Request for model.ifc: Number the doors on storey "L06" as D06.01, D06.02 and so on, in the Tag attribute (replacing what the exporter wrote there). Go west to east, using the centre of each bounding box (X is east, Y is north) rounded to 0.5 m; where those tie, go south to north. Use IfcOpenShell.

First a look at what the model holds.

```python
import ifcopenshell
import ifcopenshell.util.element
import ifcopenshell.util.placement

model = ifcopenshell.open("model.ifc")
print(model.schema)
storey = next(s for s in model.by_type("IfcBuildingStorey") if s.Name == "L06")
doors = [e for e in ifcopenshell.util.element.get_decomposition(storey) if e.is_a("IfcDoor")]
for e in sorted(doors, key=lambda e: e.id()):
    origin = ifcopenshell.util.placement.get_local_placement(e.ObjectPlacement)[:3, 3]
    print(e.id(), e.Tag, e.Name, origin.round(2) + 0.0, sep=" | ")
```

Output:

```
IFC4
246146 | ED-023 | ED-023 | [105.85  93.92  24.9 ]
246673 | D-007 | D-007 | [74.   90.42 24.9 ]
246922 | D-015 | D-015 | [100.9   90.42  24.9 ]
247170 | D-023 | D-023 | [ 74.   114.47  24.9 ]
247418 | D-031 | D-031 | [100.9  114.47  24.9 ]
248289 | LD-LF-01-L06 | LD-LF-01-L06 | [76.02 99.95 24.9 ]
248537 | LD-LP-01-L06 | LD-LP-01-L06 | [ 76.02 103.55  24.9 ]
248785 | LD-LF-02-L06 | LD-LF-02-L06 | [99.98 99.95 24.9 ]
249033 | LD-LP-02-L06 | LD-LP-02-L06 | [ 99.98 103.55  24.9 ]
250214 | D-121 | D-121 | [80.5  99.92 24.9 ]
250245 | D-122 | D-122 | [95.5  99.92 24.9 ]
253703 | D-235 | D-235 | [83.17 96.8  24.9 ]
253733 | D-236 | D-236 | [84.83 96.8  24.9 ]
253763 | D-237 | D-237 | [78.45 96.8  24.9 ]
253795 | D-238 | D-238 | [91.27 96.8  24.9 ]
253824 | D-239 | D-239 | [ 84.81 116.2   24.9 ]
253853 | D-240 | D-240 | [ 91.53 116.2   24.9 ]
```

```python
import ifcopenshell
import ifcopenshell.geom
import ifcopenshell.util.element
import ifcopenshell.util.shape

model = ifcopenshell.open("model.ifc")
settings = ifcopenshell.geom.settings()
settings.set("use-world-coords", True)


def centre(element):
    shape = ifcopenshell.geom.create_shape(settings, element)
    return ifcopenshell.util.shape.get_bbox_centroid(shape.geometry)


storey = next(s for s in model.by_type("IfcBuildingStorey") if s.Name == "L06")
doors = [e for e in ifcopenshell.util.element.get_decomposition(storey) if e.is_a("IfcDoor")]

# Insertion points can sit at a corner or the storey origin, so sort by the geometry (in metres).
centres = {e: centre(e) for e in doors}
doors.sort(key=lambda e: (round(centres[e][0] / 0.5), centres[e][1]))

for i, e in enumerate(doors, start=1):
    number = f"D06.{i:02d}"
    e.Tag = number
    print(e.id(), number)

model.write("model-out.ifc")
```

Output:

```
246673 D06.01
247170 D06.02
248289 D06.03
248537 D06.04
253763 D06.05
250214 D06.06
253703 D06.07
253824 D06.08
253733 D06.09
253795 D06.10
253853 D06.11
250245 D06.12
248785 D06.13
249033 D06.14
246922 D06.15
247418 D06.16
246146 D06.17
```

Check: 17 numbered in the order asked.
